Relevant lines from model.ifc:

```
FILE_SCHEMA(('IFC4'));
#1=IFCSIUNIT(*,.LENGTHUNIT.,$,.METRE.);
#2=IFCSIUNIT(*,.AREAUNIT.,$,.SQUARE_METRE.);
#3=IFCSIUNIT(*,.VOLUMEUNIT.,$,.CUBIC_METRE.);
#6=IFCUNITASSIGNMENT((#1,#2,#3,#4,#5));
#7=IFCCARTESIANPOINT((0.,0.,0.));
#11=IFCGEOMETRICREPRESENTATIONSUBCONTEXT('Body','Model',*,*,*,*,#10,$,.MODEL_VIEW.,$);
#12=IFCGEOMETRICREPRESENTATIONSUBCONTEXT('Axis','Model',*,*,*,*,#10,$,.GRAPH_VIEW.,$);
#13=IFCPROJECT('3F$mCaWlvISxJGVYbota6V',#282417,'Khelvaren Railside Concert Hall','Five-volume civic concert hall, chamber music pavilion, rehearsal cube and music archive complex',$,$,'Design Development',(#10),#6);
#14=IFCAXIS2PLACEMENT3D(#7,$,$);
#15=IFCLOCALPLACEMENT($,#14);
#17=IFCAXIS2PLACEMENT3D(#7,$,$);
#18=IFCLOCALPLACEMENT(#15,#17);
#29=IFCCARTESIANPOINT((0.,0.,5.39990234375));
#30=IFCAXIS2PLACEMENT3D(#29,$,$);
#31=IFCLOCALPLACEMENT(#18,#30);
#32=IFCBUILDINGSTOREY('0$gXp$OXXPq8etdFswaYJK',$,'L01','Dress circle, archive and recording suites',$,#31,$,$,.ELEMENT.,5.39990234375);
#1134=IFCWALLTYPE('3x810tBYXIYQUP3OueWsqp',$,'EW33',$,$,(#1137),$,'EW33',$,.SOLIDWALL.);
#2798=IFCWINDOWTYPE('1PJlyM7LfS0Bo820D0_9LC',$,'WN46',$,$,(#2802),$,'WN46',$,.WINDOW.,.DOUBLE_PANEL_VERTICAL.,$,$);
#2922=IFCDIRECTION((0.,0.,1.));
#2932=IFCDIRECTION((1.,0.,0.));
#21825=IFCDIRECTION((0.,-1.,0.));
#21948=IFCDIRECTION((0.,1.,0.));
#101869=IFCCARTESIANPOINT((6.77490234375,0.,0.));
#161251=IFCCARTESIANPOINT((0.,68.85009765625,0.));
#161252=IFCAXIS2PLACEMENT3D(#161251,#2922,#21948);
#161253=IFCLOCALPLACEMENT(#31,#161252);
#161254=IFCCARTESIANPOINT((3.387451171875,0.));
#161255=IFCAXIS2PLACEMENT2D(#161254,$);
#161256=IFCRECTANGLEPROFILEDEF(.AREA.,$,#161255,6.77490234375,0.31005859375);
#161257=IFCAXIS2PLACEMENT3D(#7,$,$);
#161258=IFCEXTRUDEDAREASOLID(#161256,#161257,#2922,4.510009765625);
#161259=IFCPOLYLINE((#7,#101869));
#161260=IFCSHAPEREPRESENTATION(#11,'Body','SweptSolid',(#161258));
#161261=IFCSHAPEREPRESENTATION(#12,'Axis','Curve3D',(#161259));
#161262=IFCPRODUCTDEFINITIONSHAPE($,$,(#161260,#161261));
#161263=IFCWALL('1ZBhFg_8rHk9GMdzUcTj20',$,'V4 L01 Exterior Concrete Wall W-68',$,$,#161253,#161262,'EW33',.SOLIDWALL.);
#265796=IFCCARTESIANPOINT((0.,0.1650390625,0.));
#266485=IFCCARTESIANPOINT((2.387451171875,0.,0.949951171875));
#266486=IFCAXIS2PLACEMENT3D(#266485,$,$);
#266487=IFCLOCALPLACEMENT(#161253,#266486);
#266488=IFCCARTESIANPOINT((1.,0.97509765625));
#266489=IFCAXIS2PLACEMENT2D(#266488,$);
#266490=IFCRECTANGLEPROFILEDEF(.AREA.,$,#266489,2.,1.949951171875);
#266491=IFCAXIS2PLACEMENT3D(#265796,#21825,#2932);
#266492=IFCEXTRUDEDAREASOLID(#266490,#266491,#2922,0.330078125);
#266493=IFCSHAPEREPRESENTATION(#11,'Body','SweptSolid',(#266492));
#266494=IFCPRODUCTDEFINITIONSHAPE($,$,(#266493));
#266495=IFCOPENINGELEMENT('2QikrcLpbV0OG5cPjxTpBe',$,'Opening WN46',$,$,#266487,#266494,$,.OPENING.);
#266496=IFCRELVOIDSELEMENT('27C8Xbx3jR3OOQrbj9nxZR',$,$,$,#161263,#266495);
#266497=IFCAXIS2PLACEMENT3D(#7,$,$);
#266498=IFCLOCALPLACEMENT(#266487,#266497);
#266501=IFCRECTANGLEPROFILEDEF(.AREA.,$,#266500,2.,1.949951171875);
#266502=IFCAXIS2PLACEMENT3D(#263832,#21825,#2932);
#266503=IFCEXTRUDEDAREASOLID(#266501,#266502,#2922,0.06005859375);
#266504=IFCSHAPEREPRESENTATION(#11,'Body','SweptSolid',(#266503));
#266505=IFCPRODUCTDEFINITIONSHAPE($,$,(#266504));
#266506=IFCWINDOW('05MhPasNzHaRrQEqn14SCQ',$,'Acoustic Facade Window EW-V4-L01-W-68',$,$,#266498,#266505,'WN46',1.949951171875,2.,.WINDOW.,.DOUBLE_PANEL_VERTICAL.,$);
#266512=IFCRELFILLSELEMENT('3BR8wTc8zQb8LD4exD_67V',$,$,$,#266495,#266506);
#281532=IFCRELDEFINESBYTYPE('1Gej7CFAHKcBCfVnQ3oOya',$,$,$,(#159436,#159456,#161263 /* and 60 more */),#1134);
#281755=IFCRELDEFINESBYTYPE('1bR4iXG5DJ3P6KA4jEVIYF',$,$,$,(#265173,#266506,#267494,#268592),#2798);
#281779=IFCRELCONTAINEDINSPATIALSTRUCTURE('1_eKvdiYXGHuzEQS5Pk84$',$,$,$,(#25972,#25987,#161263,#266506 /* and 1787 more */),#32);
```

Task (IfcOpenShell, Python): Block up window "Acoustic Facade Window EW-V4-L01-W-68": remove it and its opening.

```python
import ifcopenshell
import ifcopenshell.api.feature
import ifcopenshell.api.root
import ifcopenshell.geom
import ifcopenshell.util.shape

model = ifcopenshell.open("model.ifc")
settings = ifcopenshell.geom.settings()


def volume(element):
    """Net volume in cubic metres, openings subtracted."""
    shape = ifcopenshell.geom.create_shape(settings, element)
    return ifcopenshell.util.shape.get_volume(shape.geometry)


window = model.by_id(266506)
opening = window.FillsVoids[0].RelatingOpeningElement
wall = opening.VoidsElements[0].RelatingBuildingElement
before = volume(wall)

ifcopenshell.api.root.remove_product(model, product=window)
ifcopenshell.api.feature.remove_feature(model, feature=opening)

after = volume(wall)

print(f"wall volume {before:.3f} -> {after:.3f} m3")

model.write("model_v2.ifc")
```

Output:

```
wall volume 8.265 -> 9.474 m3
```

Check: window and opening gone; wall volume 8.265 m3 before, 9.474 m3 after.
